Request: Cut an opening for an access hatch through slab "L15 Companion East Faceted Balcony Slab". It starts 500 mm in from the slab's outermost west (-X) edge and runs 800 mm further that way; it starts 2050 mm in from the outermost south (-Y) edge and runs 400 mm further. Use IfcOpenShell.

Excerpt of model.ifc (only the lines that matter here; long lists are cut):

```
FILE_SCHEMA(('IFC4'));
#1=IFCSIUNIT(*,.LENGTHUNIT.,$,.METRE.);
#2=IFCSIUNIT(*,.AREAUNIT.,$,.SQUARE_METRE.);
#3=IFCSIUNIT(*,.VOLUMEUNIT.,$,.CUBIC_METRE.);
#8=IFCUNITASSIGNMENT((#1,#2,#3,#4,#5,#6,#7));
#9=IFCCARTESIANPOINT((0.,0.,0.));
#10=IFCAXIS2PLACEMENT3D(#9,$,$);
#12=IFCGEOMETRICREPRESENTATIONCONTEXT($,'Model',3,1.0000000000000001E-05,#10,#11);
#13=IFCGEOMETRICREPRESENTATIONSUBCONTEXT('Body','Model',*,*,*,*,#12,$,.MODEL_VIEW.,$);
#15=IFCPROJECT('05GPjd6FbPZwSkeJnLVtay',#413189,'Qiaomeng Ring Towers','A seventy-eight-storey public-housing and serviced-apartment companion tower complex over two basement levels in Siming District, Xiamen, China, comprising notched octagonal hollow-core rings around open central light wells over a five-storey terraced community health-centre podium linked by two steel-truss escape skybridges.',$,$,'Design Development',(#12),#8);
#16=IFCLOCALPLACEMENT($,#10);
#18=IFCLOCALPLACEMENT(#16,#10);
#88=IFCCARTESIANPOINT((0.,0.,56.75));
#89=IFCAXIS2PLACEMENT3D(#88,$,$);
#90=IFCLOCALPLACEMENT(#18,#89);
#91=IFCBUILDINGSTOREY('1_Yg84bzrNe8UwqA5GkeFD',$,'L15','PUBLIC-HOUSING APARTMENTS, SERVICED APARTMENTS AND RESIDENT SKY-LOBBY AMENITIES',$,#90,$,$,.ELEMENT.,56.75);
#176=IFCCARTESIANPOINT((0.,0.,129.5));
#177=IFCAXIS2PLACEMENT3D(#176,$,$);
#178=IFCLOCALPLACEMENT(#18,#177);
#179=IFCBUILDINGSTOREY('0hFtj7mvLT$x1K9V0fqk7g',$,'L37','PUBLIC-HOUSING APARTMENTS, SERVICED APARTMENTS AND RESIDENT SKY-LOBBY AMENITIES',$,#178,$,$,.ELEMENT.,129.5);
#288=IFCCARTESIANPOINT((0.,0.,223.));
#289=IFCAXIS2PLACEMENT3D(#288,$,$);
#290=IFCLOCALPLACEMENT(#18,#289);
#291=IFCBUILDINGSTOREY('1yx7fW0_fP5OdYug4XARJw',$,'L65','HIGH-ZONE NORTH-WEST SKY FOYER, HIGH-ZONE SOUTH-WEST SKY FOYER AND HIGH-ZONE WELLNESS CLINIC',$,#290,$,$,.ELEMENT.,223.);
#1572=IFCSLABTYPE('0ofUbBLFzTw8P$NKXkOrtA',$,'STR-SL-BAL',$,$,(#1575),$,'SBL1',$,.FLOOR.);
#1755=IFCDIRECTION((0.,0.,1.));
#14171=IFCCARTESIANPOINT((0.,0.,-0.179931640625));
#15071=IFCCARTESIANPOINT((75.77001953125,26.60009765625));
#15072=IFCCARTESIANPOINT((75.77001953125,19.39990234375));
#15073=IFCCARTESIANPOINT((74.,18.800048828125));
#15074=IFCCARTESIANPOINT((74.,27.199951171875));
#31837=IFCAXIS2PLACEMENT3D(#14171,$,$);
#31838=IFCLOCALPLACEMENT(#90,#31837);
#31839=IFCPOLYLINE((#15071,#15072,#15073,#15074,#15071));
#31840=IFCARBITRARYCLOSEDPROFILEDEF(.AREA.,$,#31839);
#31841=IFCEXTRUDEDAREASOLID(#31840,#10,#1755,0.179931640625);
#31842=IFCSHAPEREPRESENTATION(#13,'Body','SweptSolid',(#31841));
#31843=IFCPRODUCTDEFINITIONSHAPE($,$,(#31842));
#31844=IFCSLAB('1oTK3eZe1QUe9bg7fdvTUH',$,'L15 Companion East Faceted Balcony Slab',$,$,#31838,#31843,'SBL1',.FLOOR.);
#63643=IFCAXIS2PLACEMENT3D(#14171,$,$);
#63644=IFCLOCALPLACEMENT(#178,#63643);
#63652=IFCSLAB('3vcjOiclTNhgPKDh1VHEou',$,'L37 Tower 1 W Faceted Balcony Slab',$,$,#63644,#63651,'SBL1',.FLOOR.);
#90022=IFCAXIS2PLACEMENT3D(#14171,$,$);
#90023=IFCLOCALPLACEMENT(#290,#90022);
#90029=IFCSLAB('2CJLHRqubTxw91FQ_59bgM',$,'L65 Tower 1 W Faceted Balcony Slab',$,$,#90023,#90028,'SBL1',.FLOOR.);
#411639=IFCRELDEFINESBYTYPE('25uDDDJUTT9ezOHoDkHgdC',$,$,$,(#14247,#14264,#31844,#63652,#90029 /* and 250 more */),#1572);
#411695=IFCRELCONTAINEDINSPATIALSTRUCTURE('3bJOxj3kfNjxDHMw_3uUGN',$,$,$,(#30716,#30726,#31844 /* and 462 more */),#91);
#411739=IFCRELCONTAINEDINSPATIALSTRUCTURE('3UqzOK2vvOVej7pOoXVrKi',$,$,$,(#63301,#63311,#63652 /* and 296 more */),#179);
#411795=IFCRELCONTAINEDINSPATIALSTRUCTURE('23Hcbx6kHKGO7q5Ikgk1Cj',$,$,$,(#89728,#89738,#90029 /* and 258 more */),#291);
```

```python
import numpy as np
import ifcopenshell
import ifcopenshell.api.feature
import ifcopenshell.api.geometry
import ifcopenshell.api.root
import ifcopenshell.geom
import ifcopenshell.util.placement
import ifcopenshell.util.representation
import ifcopenshell.util.shape
import ifcopenshell.util.unit

model = ifcopenshell.open("model.ifc")
unit_scale = ifcopenshell.util.unit.calculate_unit_scale(model)
settings = ifcopenshell.geom.settings()


def volume(element):
    """Net volume in cubic metres, openings subtracted."""
    shape = ifcopenshell.geom.create_shape(settings, element)
    return ifcopenshell.util.shape.get_volume(shape.geometry)


slab = model.by_id(31844)
before = volume(slab)

# Extent in the slab's own axes, in metres. The edges named are its -X and -Y sides.
slab_shape = ifcopenshell.geom.create_shape(settings, slab)
vertices = ifcopenshell.util.shape.get_vertices(slab_shape.geometry)
x_min, y_min, bottom = vertices.min(axis=0)
top = vertices[:, 2].max()

opening = ifcopenshell.api.root.create_entity(model, ifc_class="IfcOpeningElement", name="Access hatch opening", predefined_type="OPENING")
context = ifcopenshell.util.representation.get_context(model, "Model", "Body", "MODEL_VIEW")
width, depth = 0.8, 0.4
outline = [(0.0, 0.0), (width, 0.0), (width, depth), (0.0, depth), (0.0, 0.0)]
# Overshoot both faces by 50 mm so the cut is clean.
shape = ifcopenshell.api.geometry.add_slab_representation(
    model, context=context, depth=top - bottom + 0.1, polyline=outline
)
ifcopenshell.api.geometry.assign_representation(model, product=opening, representation=shape)

matrix = ifcopenshell.util.placement.get_local_placement(slab.ObjectPlacement)
matrix[:, 3] = matrix @ np.append(np.array([x_min + 0.5, y_min + 2.05, bottom - 0.05]) / unit_scale, 1.0)
ifcopenshell.api.geometry.edit_object_placement(model, product=opening, matrix=matrix, is_si=False)
ifcopenshell.api.feature.add_feature(model, feature=opening, element=slab)

after = volume(slab)

print(f"slab volume {before:.3f} -> {after:.3f} m3")

model.write("model-out.ifc")
```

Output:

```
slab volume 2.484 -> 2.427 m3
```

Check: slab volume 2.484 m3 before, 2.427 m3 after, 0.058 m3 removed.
